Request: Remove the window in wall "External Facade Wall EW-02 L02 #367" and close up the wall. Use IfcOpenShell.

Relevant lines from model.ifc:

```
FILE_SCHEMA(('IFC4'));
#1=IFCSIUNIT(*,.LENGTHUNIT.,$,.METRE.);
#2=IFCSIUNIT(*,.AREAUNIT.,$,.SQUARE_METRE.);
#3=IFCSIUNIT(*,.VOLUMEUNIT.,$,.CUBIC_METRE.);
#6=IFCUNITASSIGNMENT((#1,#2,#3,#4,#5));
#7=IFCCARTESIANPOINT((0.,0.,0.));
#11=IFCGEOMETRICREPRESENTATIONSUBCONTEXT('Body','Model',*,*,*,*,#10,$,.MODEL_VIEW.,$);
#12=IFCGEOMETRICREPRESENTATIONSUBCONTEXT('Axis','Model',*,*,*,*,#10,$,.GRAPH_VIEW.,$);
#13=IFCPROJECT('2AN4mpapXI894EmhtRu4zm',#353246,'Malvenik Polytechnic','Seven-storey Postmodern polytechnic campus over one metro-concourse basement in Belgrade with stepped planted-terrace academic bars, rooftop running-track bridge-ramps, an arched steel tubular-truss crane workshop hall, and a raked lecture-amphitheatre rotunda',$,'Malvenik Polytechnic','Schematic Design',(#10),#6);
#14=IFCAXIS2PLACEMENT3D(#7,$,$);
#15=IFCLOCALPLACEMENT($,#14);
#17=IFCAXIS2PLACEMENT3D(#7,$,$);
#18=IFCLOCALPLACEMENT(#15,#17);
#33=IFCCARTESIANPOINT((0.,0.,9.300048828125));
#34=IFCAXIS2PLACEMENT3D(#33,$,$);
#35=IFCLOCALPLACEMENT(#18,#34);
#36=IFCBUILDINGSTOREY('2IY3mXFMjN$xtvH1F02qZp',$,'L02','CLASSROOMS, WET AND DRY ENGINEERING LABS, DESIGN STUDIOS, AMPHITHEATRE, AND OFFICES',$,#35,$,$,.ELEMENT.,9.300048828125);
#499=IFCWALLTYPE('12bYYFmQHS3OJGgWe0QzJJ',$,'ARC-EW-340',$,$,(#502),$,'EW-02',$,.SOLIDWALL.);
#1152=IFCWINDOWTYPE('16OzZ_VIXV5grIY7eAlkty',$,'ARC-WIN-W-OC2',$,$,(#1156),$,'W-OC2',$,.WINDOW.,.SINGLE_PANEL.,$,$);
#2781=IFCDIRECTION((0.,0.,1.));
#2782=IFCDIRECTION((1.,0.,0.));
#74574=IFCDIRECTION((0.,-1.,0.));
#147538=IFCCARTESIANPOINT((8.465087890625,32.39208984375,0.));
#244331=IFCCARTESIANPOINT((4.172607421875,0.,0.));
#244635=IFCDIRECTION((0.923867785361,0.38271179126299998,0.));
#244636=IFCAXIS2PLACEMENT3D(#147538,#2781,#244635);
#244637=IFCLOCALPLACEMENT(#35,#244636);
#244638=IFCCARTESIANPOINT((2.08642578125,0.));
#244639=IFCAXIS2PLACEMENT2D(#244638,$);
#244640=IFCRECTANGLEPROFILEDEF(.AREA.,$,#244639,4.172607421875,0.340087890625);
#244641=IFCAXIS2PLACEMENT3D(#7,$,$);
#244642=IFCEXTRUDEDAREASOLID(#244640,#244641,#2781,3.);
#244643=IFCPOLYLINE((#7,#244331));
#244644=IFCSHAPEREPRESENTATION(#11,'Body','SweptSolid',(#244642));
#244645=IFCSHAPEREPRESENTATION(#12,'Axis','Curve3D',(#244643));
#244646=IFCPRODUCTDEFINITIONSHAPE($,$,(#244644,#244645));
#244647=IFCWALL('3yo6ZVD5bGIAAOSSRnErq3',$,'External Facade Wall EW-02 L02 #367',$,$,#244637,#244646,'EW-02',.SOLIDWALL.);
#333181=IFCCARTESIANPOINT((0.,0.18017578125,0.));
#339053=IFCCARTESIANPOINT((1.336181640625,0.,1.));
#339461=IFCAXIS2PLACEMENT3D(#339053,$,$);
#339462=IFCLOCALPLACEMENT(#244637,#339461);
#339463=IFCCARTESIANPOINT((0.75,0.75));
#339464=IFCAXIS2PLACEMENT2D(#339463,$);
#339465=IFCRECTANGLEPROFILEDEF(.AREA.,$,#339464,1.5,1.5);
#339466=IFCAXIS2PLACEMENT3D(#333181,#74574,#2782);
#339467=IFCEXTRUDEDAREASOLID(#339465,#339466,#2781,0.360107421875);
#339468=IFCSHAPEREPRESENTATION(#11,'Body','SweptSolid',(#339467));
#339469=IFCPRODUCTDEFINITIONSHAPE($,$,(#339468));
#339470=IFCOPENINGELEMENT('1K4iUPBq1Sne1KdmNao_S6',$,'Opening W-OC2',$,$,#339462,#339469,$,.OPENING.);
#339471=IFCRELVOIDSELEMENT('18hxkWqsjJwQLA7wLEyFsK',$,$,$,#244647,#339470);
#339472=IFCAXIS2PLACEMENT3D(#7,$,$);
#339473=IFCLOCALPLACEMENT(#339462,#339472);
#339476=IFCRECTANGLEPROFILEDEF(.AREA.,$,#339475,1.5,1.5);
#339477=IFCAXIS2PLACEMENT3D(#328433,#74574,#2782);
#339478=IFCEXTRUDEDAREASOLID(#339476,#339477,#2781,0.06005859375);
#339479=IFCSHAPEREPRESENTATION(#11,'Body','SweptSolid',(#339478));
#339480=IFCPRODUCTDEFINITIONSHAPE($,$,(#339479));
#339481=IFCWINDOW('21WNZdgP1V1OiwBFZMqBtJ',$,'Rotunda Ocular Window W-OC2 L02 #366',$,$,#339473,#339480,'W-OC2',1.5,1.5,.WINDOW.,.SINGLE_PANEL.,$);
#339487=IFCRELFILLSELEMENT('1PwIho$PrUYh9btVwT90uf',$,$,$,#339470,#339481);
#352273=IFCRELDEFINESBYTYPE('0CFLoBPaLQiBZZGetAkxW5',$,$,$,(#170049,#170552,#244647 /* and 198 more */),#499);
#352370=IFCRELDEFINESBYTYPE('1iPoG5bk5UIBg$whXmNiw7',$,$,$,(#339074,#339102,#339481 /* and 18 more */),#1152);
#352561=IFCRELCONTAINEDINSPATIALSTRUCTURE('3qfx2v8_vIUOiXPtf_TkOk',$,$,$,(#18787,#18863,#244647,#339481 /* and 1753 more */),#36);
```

```python
import ifcopenshell
import ifcopenshell.api.feature
import ifcopenshell.api.root
import ifcopenshell.geom
import ifcopenshell.util.shape

model = ifcopenshell.open("model.ifc")
settings = ifcopenshell.geom.settings()


def volume(element):
    """Net volume in cubic metres, openings subtracted."""
    shape = ifcopenshell.geom.create_shape(settings, element)
    return ifcopenshell.util.shape.get_volume(shape.geometry)


window = model.by_guid("21WNZdgP1V1OiwBFZMqBtJ")
opening = window.FillsVoids[0].RelatingOpeningElement
wall = opening.VoidsElements[0].RelatingBuildingElement
before = volume(wall)

ifcopenshell.api.root.remove_product(model, product=window)
ifcopenshell.api.feature.remove_feature(model, feature=opening)

after = volume(wall)

print(f"wall volume {before:.3f} -> {after:.3f} m3")

model.write("model-out.ifc")
```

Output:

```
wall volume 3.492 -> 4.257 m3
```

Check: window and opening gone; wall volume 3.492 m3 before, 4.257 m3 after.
